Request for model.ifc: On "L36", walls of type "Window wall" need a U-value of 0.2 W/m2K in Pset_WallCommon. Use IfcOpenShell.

First a look at what the model holds.

```python
import ifcopenshell
import ifcopenshell.util.element

model = ifcopenshell.open("model.ifc")
print(model.schema)
storey = next(s for s in model.by_type("IfcBuildingStorey") if s.Name == "L36")
walls = [e for e in ifcopenshell.util.element.get_decomposition(storey) if e.is_a("IfcWall")]
seen = {}
for e in walls:
    element_type = ifcopenshell.util.element.get_type(e)
    key = (element_type.Name if element_type != e and element_type else None, ifcopenshell.util.element.get_pset(e, "Pset_WallCommon", "ThermalTransmittance"))
    seen[key] = seen.get(key, 0) + 1
for (name, value), count in sorted(seen.items(), key=str):
    print(count, "x", name, "|", value)
```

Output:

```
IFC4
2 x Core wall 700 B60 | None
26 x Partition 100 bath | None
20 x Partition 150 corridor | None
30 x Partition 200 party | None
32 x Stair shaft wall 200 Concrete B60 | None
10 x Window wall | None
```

```python
import ifcopenshell
import ifcopenshell.api.pset
import ifcopenshell.util.element

model = ifcopenshell.open("model.ifc")

storey = next(s for s in model.by_type("IfcBuildingStorey") if s.Name == "L36")
walls = [e for e in ifcopenshell.util.element.get_decomposition(storey) if e.is_a("IfcWall")]

count = 0
for e in walls:
    element_type = ifcopenshell.util.element.get_type(e)
    if element_type in (None, e) or element_type.Name != "Window wall":
        continue
    found = ifcopenshell.util.element.get_pset(e, "Pset_WallCommon", should_inherit=False)
    if found:
        pset = model.by_id(found["id"])
        if len(ifcopenshell.util.element.get_elements_by_pset(pset)) > 1:
            pset = ifcopenshell.api.pset.unshare_pset(model, products=[e], pset=pset)[0]
    else:
        pset = ifcopenshell.api.pset.add_pset(model, product=e, name="Pset_WallCommon")
    ifcopenshell.api.pset.edit_pset(model, pset=pset, properties={"ThermalTransmittance": 0.2})
    count += 1

print(count, "walls updated")

model.write("model-out.ifc")
```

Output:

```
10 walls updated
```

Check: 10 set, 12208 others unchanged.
